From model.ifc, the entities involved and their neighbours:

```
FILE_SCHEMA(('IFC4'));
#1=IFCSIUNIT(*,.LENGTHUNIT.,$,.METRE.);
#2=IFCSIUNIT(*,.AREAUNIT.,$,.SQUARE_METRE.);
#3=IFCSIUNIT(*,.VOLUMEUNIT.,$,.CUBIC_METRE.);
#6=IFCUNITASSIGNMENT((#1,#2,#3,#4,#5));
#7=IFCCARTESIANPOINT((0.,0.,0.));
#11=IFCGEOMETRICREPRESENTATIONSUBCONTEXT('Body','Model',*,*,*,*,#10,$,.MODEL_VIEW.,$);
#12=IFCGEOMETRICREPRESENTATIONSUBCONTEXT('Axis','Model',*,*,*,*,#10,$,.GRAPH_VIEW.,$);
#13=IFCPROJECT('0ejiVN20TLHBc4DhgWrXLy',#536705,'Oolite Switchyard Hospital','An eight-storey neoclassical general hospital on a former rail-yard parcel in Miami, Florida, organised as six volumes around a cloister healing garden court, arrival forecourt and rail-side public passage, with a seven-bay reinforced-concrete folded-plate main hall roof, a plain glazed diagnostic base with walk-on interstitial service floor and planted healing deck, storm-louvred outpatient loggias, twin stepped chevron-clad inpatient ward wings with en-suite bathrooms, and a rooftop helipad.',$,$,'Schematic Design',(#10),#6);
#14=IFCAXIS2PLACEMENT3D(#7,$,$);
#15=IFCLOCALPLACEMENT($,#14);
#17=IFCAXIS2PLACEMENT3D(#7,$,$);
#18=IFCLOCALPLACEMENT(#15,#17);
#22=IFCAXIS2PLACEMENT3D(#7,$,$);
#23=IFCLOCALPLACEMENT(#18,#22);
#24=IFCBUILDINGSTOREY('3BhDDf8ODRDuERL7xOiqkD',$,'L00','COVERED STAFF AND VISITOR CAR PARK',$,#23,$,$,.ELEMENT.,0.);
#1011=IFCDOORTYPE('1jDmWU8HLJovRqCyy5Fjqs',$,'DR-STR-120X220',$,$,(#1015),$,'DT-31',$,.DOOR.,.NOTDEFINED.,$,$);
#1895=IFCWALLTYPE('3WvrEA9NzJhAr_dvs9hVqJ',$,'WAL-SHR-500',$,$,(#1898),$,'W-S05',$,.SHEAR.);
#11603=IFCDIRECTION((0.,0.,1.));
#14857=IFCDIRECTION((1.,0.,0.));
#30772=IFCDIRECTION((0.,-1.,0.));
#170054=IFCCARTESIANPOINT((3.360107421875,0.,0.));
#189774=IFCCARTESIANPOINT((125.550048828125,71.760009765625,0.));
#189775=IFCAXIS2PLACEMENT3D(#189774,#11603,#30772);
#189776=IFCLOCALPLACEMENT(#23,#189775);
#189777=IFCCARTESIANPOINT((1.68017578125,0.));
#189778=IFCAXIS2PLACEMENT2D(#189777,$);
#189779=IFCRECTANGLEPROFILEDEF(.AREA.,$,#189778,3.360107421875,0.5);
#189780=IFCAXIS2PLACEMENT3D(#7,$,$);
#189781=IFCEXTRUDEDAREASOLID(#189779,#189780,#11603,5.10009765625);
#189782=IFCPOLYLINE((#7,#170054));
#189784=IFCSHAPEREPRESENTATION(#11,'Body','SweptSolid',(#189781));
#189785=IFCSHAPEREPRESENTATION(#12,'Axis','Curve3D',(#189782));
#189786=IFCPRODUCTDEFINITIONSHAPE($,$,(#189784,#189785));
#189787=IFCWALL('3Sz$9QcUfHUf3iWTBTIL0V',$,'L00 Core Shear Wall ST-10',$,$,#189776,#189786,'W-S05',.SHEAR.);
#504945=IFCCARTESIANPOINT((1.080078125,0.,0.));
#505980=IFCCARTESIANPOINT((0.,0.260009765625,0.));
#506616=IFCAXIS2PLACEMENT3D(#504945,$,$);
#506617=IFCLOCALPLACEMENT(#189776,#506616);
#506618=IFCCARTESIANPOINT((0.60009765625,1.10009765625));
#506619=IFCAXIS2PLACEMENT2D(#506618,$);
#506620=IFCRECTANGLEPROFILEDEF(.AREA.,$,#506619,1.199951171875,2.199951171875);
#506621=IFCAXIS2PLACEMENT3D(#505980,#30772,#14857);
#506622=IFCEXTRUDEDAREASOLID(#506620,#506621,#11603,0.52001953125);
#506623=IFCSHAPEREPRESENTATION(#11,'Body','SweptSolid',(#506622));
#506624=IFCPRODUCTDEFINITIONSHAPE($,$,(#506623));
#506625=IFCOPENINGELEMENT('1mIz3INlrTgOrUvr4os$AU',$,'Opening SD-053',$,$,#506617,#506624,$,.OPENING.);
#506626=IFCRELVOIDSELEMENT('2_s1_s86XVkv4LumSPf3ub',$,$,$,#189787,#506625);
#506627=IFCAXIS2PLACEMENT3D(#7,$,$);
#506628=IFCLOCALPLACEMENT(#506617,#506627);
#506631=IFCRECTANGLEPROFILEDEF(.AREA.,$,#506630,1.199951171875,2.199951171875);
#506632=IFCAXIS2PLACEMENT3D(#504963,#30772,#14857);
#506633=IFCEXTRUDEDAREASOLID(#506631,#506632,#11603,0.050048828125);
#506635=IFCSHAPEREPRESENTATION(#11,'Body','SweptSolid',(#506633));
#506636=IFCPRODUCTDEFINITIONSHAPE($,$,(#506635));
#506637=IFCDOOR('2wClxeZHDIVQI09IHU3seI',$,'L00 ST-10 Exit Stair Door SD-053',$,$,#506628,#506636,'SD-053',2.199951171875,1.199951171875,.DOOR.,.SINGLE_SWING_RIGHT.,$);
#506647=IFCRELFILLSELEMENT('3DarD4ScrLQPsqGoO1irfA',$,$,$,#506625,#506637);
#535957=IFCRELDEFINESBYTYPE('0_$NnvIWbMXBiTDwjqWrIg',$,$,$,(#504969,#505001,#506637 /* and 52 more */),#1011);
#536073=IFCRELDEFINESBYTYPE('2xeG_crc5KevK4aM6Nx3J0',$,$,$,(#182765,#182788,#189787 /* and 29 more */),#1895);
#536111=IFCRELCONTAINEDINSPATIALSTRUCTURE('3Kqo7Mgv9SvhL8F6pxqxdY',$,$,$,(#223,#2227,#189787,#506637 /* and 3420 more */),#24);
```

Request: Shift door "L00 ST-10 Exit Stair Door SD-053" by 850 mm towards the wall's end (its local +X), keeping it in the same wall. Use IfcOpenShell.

```python
import ifcopenshell
import ifcopenshell.api.geometry
import ifcopenshell.util.placement

model = ifcopenshell.open("model.ifc")

door = model.by_guid("2wClxeZHDIVQI09IHU3seI")
opening = door.FillsVoids[0].RelatingOpeningElement
wall = opening.VoidsElements[0].RelatingBuildingElement

wall_matrix = ifcopenshell.util.placement.get_local_placement(wall.ObjectPlacement)
shift = wall_matrix[:3, 0] * 0.85
before = ifcopenshell.util.placement.get_local_placement(door.ObjectPlacement)[:3, 3].copy()

# The door is placed relative to its opening, so it follows when the opening moves.
matrix = ifcopenshell.util.placement.get_local_placement(opening.ObjectPlacement)
matrix[:3, 3] += shift
ifcopenshell.api.geometry.edit_object_placement(
    model, product=opening, matrix=matrix, is_si=False, should_transform_children=True
)

after = ifcopenshell.util.placement.get_local_placement(door.ObjectPlacement)[:3, 3]
print("door moved by", (after - before).round(3) + 0.0)

model.write("model_edited.ifc")
```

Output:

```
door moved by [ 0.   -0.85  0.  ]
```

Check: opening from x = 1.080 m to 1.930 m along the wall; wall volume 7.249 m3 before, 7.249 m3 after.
